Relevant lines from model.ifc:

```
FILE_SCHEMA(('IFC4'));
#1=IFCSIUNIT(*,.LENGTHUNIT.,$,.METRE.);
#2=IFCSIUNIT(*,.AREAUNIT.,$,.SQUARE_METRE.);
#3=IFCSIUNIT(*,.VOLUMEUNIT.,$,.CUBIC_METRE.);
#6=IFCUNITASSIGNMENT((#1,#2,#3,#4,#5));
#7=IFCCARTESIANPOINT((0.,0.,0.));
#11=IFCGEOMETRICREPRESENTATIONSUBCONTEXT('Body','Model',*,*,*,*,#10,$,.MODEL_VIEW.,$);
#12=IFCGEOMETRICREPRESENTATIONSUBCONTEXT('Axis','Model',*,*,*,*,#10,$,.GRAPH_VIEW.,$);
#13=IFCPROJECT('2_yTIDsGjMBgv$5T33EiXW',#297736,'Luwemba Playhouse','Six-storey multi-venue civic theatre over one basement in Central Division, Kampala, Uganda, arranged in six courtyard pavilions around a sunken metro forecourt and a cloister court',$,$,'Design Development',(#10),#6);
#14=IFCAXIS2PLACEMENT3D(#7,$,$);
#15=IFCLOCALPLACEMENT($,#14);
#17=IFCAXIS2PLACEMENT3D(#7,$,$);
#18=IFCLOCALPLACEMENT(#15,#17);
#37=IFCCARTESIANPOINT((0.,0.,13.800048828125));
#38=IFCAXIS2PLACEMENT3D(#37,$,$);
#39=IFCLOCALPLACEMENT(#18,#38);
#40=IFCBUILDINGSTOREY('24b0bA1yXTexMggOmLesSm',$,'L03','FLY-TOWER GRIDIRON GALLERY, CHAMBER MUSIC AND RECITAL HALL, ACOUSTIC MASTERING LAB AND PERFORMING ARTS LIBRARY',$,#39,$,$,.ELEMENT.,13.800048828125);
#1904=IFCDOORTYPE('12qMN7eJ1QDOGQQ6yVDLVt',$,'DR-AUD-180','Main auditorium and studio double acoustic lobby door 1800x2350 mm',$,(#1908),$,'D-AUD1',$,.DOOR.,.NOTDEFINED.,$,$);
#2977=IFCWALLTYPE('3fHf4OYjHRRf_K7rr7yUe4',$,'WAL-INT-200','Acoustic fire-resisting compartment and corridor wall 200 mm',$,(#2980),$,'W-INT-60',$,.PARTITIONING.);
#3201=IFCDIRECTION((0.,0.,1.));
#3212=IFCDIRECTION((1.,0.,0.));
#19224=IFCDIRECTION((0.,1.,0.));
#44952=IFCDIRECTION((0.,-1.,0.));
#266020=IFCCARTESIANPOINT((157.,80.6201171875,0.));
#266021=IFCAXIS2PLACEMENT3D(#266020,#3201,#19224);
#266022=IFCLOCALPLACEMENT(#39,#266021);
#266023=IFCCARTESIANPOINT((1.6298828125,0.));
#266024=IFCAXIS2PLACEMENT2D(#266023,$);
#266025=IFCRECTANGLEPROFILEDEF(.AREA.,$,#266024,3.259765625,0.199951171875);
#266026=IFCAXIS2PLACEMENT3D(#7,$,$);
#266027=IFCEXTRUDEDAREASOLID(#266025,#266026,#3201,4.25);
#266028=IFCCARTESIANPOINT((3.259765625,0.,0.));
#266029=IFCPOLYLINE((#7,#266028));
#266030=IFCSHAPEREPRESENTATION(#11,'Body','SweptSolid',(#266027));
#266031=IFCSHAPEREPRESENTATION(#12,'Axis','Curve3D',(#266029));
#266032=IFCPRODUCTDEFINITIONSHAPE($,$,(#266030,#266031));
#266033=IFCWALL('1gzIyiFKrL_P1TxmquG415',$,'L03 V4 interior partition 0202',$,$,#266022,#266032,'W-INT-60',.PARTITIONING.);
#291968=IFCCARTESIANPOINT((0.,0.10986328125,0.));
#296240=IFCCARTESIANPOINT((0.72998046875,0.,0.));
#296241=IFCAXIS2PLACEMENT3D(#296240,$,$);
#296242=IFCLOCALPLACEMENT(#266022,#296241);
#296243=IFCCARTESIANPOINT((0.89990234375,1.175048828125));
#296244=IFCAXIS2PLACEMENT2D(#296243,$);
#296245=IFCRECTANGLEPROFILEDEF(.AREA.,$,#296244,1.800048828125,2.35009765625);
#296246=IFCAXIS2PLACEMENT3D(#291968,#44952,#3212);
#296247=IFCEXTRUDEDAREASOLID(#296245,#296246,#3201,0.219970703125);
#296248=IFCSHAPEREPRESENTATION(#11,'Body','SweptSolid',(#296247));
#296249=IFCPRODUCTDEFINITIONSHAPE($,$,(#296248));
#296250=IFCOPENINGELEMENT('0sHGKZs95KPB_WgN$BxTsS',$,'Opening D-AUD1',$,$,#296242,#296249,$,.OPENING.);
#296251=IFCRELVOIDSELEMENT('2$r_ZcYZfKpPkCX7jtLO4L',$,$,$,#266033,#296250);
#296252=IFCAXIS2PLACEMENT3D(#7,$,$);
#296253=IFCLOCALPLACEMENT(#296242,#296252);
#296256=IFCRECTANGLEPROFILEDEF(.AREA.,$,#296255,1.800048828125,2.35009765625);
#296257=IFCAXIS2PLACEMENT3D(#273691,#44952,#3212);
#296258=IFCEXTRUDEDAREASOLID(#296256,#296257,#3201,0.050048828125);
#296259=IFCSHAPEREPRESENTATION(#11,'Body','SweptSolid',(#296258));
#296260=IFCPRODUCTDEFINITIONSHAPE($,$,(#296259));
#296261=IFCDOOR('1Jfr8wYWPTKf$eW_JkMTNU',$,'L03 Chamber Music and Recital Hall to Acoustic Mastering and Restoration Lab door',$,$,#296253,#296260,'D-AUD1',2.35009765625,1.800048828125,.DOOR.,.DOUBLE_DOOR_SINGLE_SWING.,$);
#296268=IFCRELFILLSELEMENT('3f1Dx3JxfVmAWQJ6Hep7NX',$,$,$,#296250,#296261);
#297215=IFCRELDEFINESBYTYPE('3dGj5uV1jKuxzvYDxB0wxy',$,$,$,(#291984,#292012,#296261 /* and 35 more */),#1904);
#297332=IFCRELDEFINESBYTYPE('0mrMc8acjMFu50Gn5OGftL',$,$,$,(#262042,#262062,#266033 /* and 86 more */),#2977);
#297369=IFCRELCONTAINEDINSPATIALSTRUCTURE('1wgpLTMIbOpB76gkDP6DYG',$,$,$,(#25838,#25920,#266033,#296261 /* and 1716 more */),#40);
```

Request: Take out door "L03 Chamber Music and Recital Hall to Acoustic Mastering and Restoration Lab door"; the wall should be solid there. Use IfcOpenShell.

```python
import ifcopenshell
import ifcopenshell.api.feature
import ifcopenshell.api.root
import ifcopenshell.geom
import ifcopenshell.util.shape

model = ifcopenshell.open("model.ifc")
settings = ifcopenshell.geom.settings()


def volume(element):
    """Net volume in cubic metres, openings subtracted."""
    shape = ifcopenshell.geom.create_shape(settings, element)
    return ifcopenshell.util.shape.get_volume(shape.geometry)


door = model.by_guid("1Jfr8wYWPTKf$eW_JkMTNU")
opening = door.FillsVoids[0].RelatingOpeningElement
wall = opening.VoidsElements[0].RelatingBuildingElement
before = volume(wall)

ifcopenshell.api.root.remove_product(model, product=door)
ifcopenshell.api.feature.remove_feature(model, feature=opening)

after = volume(wall)

print(f"wall volume {before:.3f} -> {after:.3f} m3")

model.write("model_rev.ifc")
```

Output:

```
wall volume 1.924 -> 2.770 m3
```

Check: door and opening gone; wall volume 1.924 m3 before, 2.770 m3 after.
